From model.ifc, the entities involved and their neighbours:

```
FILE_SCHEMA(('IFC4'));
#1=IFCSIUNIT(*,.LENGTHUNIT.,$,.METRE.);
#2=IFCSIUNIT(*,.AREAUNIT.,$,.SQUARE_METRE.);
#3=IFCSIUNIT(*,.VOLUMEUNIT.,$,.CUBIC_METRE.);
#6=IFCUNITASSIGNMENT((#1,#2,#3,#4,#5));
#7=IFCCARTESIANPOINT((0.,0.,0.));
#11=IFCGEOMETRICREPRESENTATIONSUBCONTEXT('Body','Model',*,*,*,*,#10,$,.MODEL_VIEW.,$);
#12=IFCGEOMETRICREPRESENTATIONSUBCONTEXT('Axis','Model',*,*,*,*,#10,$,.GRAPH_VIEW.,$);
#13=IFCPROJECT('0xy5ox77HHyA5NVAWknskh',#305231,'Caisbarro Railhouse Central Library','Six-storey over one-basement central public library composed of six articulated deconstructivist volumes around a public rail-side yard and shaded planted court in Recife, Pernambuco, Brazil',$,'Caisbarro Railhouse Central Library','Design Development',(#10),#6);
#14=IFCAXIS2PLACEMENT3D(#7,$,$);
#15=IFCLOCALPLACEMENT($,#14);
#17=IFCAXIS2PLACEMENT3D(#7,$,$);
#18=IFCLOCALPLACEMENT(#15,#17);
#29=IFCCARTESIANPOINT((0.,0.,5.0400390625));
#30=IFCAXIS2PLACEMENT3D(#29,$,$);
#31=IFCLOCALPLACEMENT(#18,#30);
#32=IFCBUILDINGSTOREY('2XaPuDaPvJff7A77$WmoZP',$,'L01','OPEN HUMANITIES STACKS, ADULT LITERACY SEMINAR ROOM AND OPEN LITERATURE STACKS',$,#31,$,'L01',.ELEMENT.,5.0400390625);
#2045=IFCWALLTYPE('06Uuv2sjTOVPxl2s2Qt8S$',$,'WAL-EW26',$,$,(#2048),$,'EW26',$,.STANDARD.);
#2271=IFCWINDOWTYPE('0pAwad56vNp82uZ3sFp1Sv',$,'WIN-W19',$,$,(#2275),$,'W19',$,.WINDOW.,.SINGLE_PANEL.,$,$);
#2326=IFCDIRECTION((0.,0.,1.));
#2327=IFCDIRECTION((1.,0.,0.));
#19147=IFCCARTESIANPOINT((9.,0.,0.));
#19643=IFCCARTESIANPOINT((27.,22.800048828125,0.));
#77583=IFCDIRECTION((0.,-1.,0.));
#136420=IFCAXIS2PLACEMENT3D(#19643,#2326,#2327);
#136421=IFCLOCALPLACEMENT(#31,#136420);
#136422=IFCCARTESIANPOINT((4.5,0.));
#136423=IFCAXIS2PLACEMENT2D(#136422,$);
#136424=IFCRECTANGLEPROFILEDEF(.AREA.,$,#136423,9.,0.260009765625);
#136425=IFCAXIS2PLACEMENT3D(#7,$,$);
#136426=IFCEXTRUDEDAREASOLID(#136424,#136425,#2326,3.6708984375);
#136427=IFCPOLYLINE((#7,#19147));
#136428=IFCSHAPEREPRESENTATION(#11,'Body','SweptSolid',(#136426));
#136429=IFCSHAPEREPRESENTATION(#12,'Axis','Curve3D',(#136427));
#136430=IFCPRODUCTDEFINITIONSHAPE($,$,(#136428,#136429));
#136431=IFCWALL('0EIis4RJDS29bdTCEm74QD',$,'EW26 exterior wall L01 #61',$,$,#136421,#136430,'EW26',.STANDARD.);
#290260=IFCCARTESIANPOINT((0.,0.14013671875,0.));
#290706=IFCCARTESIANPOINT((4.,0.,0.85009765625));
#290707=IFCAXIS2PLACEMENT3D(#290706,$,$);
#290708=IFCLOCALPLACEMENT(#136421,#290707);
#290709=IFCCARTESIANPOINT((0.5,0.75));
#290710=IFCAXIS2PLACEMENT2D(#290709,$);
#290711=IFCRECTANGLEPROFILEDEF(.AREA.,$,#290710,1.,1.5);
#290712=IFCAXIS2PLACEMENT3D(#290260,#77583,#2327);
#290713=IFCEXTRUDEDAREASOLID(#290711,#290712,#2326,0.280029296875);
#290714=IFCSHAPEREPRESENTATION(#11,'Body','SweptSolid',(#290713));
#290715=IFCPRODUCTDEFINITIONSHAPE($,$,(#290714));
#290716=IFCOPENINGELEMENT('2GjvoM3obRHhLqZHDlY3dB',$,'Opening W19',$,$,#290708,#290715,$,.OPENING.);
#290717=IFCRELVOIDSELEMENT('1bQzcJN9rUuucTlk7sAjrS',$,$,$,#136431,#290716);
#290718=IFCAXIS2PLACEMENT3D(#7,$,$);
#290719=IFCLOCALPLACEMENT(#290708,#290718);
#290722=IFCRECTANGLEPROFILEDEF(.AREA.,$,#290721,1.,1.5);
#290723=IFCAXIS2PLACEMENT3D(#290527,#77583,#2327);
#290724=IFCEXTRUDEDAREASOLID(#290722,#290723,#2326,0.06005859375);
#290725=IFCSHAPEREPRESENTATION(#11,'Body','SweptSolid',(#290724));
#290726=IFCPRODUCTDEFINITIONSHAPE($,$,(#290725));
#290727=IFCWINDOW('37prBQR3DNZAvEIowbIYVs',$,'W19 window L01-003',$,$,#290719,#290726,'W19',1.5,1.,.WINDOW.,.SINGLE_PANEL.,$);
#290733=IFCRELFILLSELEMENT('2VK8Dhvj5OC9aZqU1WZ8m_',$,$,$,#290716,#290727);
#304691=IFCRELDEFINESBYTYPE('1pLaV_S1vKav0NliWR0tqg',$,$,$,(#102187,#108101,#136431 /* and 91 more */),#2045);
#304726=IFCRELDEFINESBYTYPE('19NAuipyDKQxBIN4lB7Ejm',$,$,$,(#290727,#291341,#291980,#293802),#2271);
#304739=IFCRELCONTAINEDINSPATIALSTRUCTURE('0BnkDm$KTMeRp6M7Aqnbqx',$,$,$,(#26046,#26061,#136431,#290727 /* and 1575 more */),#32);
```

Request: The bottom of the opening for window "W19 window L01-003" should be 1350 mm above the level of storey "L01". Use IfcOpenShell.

```python
import numpy as np
import ifcopenshell
import ifcopenshell.api.geometry
import ifcopenshell.geom
import ifcopenshell.util.element
import ifcopenshell.util.placement
import ifcopenshell.util.shape
import ifcopenshell.util.unit

model = ifcopenshell.open("model.ifc")
unit_scale = ifcopenshell.util.unit.calculate_unit_scale(model)

window = model.by_guid("37prBQR3DNZAvEIowbIYVs")
opening = window.FillsVoids[0].RelatingOpeningElement
storey = ifcopenshell.util.element.get_container(window, ifc_class="IfcBuildingStorey")
level = ifcopenshell.util.placement.get_local_placement(storey.ObjectPlacement)[2, 3]

# The opening's origin need not be at the sill, so measure its lowest point.
shape = ifcopenshell.geom.create_shape(ifcopenshell.geom.settings(), opening)
bottom = ifcopenshell.util.shape.get_shape_bottom_elevation(shape, shape.geometry) / unit_scale
dz = level + 1.35 / unit_scale - bottom

shift = np.array([0.0, 0.0, dz])
# The window is placed relative to its opening, so it follows when the opening moves.
matrix = ifcopenshell.util.placement.get_local_placement(opening.ObjectPlacement)
matrix[:3, 3] += shift
ifcopenshell.api.geometry.edit_object_placement(
    model, product=opening, matrix=matrix, is_si=False, should_transform_children=True
)

print(f"moved by {dz * unit_scale:+.3f} m")

model.write("model-out.ifc")
```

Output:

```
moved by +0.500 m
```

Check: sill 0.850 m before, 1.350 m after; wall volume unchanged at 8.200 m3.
